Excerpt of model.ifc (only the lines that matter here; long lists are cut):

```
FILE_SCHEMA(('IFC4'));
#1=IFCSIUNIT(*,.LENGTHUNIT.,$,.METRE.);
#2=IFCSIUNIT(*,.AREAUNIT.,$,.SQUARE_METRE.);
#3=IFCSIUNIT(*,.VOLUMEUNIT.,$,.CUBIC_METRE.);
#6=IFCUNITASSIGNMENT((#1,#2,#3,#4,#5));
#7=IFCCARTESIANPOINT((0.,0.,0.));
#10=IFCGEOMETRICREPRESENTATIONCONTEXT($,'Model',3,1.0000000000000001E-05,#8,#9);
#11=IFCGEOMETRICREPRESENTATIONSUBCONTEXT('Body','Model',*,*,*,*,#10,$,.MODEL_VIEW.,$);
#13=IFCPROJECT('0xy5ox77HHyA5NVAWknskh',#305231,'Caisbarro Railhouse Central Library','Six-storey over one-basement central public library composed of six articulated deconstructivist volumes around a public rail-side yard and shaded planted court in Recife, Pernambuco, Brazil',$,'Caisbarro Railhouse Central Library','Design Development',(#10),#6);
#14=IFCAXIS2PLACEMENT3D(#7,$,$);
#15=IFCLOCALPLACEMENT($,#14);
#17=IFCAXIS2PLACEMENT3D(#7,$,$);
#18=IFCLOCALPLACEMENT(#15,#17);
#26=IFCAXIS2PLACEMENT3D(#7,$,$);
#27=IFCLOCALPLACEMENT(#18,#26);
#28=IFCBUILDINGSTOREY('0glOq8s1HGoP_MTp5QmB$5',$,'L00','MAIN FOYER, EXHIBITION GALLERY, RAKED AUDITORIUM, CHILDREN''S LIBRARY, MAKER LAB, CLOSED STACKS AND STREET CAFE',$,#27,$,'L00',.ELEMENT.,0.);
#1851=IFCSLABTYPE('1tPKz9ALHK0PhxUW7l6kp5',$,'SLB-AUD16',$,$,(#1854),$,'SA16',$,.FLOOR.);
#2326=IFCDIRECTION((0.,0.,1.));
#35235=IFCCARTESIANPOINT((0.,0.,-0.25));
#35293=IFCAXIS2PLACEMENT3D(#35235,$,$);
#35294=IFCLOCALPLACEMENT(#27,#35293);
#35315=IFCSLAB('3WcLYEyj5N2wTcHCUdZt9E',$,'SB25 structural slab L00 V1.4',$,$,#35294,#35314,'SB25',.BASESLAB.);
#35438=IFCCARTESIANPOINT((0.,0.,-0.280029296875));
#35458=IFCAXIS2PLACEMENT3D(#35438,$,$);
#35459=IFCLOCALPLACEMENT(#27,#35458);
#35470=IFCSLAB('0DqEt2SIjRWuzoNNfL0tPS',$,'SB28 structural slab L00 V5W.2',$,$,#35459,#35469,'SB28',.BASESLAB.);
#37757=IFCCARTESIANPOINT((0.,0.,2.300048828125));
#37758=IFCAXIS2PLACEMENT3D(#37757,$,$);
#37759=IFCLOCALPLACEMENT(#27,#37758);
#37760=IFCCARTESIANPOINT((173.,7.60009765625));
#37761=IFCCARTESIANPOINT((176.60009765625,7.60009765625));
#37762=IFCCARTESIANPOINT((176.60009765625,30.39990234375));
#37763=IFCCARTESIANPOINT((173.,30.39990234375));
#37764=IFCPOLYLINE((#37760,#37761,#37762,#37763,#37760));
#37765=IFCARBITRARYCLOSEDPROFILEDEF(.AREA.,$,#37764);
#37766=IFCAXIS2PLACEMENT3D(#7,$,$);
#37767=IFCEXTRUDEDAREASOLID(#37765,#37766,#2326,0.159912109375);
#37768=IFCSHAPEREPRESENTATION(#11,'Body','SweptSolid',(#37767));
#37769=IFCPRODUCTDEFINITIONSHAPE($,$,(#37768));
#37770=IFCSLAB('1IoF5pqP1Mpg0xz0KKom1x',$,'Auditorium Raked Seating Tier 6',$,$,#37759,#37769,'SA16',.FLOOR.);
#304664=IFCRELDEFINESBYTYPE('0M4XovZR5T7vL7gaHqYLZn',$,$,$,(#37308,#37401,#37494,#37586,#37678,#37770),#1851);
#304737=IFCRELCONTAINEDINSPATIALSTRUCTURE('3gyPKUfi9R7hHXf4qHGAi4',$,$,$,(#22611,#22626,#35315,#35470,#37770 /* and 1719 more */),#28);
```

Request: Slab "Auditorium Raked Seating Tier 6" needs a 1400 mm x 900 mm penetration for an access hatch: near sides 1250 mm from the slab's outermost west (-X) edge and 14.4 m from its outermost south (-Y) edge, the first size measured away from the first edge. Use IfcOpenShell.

```python
import numpy as np
import ifcopenshell
import ifcopenshell.api.feature
import ifcopenshell.api.geometry
import ifcopenshell.api.root
import ifcopenshell.geom
import ifcopenshell.util.placement
import ifcopenshell.util.representation
import ifcopenshell.util.shape
import ifcopenshell.util.unit

model = ifcopenshell.open("model.ifc")
unit_scale = ifcopenshell.util.unit.calculate_unit_scale(model)
settings = ifcopenshell.geom.settings()


def volume(element):
    """Net volume in cubic metres, openings subtracted."""
    shape = ifcopenshell.geom.create_shape(settings, element)
    return ifcopenshell.util.shape.get_volume(shape.geometry)


slab = model.by_guid("1IoF5pqP1Mpg0xz0KKom1x")
before = volume(slab)

# Extent in the slab's own axes, in metres. The edges named are its -X and -Y sides.
slab_shape = ifcopenshell.geom.create_shape(settings, slab)
vertices = ifcopenshell.util.shape.get_vertices(slab_shape.geometry)
x_min, y_min, bottom = vertices.min(axis=0)
top = vertices[:, 2].max()

opening = ifcopenshell.api.root.create_entity(model, ifc_class="IfcOpeningElement", name="Access hatch opening", predefined_type="OPENING")
context = ifcopenshell.util.representation.get_context(model, "Model", "Body", "MODEL_VIEW")
width, depth = 1.4, 0.9
outline = [(0.0, 0.0), (width, 0.0), (width, depth), (0.0, depth), (0.0, 0.0)]
# Overshoot both faces by 50 mm so the cut is clean.
shape = ifcopenshell.api.geometry.add_slab_representation(
    model, context=context, depth=top - bottom + 0.1, polyline=outline
)
ifcopenshell.api.geometry.assign_representation(model, product=opening, representation=shape)

matrix = ifcopenshell.util.placement.get_local_placement(slab.ObjectPlacement)
matrix[:, 3] = matrix @ np.append(np.array([x_min + 1.25, y_min + 14.4, bottom - 0.05]) / unit_scale, 1.0)
ifcopenshell.api.geometry.edit_object_placement(model, product=opening, matrix=matrix, is_si=False)
ifcopenshell.api.feature.add_feature(model, feature=opening, element=slab)

after = volume(slab)

print(f"slab volume {before:.3f} -> {after:.3f} m3")

model.write("model_v2.ifc")
```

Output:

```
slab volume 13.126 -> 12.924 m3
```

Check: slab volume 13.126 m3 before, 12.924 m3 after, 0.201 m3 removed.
